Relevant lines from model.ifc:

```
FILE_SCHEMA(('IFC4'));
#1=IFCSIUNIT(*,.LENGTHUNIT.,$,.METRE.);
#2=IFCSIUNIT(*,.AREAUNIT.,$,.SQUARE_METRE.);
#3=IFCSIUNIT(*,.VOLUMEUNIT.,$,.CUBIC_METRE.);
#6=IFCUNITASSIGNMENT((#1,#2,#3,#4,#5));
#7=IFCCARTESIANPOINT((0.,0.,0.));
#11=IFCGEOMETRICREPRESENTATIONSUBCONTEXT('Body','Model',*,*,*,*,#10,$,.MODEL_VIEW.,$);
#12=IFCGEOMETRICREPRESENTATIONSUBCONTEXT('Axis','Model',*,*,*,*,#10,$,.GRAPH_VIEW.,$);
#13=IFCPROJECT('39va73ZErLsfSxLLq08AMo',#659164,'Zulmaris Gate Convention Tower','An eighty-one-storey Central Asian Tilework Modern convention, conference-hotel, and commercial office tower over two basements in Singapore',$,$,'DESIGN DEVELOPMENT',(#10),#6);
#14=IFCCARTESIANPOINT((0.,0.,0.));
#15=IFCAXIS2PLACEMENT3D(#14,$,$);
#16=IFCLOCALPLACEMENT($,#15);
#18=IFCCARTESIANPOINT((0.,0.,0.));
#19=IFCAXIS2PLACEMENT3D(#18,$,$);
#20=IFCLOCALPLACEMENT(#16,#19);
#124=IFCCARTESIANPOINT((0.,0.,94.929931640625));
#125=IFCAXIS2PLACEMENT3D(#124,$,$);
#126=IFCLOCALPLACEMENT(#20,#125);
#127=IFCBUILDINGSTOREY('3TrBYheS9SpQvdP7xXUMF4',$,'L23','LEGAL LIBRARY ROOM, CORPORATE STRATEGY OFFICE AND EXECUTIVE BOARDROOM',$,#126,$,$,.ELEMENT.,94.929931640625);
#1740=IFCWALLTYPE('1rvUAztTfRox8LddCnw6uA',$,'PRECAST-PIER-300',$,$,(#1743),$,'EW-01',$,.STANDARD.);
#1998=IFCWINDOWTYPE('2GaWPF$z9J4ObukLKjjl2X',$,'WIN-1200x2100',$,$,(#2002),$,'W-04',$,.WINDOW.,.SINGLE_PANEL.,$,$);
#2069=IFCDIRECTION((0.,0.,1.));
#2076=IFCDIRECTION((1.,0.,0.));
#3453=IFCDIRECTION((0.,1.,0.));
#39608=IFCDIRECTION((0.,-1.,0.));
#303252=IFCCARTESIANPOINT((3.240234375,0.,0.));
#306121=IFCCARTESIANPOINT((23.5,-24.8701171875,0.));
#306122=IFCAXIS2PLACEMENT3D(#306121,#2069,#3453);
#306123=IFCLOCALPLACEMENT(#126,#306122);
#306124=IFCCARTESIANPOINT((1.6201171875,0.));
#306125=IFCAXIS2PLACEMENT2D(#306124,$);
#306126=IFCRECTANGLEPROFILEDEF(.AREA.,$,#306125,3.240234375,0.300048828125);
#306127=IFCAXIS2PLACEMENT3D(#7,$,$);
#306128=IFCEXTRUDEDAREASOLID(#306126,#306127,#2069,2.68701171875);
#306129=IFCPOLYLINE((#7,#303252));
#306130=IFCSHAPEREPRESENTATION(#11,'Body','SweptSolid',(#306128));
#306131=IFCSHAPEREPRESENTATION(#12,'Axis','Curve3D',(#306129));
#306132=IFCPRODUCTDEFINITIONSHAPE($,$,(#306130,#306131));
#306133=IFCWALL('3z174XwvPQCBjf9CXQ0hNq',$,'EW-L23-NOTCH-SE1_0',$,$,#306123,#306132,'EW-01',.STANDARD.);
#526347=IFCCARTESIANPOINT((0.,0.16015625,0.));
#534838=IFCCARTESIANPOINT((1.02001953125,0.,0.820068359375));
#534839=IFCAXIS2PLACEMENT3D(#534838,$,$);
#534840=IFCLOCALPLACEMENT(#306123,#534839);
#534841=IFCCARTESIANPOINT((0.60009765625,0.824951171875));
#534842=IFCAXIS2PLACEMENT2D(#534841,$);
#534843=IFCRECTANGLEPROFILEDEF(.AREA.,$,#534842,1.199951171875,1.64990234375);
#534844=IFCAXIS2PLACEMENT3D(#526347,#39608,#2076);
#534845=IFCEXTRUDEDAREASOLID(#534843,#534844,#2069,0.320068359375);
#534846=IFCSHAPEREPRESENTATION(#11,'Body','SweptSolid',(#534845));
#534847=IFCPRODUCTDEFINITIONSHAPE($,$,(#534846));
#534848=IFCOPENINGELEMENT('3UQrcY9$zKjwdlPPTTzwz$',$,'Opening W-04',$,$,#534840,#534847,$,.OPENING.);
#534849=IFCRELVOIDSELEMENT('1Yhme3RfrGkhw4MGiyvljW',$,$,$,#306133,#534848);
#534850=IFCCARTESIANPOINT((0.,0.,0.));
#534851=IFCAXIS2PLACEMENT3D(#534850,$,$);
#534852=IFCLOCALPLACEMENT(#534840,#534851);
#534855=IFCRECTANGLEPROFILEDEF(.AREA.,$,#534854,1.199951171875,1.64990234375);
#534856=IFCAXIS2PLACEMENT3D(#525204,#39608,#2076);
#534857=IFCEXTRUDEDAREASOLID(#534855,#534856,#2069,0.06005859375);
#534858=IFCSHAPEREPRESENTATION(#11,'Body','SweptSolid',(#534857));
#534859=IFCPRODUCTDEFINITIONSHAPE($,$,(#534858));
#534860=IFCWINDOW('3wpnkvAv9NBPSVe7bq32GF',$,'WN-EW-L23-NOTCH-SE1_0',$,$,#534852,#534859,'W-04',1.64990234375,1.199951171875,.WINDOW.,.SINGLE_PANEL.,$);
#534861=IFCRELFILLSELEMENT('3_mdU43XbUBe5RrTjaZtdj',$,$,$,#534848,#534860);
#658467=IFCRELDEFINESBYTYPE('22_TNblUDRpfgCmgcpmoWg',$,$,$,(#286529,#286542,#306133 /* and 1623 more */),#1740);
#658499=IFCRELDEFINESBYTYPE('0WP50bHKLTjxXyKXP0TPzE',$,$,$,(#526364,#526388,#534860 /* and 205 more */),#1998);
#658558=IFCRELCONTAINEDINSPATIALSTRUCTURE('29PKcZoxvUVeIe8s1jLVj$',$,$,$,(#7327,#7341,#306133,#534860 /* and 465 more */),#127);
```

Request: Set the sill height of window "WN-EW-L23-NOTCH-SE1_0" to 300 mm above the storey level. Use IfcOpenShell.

```python
import numpy as np
import ifcopenshell
import ifcopenshell.api.geometry
import ifcopenshell.geom
import ifcopenshell.util.element
import ifcopenshell.util.placement
import ifcopenshell.util.shape
import ifcopenshell.util.unit

model = ifcopenshell.open("model.ifc")
unit_scale = ifcopenshell.util.unit.calculate_unit_scale(model)

window = model.by_guid("3wpnkvAv9NBPSVe7bq32GF")
opening = window.FillsVoids[0].RelatingOpeningElement
storey = ifcopenshell.util.element.get_container(window, ifc_class="IfcBuildingStorey")
level = ifcopenshell.util.placement.get_local_placement(storey.ObjectPlacement)[2, 3]

# The opening's origin need not be at the sill, so measure its lowest point.
shape = ifcopenshell.geom.create_shape(ifcopenshell.geom.settings(), opening)
bottom = ifcopenshell.util.shape.get_shape_bottom_elevation(shape, shape.geometry) / unit_scale
dz = level + 0.3 / unit_scale - bottom

shift = np.array([0.0, 0.0, dz])
# The window is placed relative to its opening, so it follows when the opening moves.
matrix = ifcopenshell.util.placement.get_local_placement(opening.ObjectPlacement)
matrix[:3, 3] += shift
ifcopenshell.api.geometry.edit_object_placement(
    model, product=opening, matrix=matrix, is_si=False, should_transform_children=True
)

print(f"moved by {dz * unit_scale:+.3f} m")

model.write("model-out.ifc")
```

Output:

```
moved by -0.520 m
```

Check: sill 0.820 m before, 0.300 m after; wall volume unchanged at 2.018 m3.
